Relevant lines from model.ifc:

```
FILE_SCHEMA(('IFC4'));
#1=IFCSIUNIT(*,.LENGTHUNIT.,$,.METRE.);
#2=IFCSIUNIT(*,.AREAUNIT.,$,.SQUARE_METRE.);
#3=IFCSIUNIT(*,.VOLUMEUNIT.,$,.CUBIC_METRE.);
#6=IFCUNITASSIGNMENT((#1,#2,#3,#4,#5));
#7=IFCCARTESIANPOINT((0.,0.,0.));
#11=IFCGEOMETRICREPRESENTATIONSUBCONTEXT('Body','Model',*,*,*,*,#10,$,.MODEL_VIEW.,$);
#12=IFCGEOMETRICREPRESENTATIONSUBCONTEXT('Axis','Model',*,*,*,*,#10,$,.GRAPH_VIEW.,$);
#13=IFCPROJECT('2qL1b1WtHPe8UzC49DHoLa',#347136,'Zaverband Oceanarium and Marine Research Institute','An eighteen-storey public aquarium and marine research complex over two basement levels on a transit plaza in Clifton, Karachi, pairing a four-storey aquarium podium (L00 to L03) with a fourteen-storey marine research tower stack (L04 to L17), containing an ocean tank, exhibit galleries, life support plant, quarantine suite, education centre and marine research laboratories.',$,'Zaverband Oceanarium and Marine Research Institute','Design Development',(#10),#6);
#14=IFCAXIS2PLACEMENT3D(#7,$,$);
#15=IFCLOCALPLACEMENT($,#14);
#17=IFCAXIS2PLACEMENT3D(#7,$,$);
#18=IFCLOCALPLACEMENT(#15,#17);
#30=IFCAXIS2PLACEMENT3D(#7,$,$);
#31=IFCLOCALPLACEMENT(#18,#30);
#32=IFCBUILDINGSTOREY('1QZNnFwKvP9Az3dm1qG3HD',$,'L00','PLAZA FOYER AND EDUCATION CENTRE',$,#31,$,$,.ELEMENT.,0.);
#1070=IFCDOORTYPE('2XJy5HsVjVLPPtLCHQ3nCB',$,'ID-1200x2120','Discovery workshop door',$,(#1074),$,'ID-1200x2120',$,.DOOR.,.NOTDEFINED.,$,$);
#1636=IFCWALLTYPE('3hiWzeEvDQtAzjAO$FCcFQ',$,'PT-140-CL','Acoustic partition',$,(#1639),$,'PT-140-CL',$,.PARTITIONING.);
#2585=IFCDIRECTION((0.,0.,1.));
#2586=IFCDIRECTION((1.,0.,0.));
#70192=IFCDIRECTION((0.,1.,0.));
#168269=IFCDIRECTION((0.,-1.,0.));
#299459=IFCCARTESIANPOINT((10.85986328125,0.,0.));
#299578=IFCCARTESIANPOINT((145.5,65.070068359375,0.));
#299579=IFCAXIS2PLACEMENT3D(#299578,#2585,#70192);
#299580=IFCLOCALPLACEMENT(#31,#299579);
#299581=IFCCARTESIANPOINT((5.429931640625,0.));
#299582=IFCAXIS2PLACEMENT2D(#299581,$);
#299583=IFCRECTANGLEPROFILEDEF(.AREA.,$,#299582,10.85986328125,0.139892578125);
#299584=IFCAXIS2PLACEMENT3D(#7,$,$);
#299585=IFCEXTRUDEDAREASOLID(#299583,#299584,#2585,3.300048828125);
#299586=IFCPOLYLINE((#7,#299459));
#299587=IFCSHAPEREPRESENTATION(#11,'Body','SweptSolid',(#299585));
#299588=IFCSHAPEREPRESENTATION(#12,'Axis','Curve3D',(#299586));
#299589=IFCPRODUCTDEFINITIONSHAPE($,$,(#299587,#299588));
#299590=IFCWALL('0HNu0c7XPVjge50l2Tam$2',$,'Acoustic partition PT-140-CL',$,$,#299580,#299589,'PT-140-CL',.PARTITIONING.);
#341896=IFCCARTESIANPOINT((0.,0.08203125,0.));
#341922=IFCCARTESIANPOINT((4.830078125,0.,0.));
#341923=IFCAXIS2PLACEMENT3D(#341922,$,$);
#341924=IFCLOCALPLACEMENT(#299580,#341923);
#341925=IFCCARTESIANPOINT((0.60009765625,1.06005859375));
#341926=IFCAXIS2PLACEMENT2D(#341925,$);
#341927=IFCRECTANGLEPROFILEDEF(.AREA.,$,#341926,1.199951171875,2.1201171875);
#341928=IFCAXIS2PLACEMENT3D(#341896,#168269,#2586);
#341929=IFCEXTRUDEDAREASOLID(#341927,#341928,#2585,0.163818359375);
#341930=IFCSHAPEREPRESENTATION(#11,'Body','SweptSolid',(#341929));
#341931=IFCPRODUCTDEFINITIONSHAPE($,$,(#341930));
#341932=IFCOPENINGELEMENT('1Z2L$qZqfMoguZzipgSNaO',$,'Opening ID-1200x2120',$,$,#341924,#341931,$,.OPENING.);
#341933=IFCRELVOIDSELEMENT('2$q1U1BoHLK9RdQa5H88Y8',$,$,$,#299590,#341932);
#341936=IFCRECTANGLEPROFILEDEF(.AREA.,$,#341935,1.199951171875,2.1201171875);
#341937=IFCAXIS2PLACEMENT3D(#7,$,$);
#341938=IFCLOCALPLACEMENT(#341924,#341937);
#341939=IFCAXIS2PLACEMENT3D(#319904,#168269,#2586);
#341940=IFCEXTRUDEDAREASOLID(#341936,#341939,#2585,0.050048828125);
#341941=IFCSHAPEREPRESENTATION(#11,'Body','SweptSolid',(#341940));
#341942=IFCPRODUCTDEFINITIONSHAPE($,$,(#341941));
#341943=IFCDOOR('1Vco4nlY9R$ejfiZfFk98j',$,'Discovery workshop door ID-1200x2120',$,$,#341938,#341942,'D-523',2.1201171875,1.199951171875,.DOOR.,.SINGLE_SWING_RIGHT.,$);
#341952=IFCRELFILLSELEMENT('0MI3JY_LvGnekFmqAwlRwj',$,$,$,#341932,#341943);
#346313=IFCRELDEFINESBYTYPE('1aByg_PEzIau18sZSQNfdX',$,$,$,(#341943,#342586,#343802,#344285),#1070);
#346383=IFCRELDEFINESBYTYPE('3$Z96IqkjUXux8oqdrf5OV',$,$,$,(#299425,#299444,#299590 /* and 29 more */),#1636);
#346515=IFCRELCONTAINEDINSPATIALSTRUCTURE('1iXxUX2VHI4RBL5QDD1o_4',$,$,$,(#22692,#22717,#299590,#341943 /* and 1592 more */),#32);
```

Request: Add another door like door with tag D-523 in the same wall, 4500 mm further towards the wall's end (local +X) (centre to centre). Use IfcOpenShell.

```python
import ifcopenshell
import ifcopenshell.api.feature
import ifcopenshell.api.geometry
import ifcopenshell.api.root
import ifcopenshell.geom
import ifcopenshell.util.element
import ifcopenshell.util.placement
import ifcopenshell.util.shape
import ifcopenshell.util.unit

model = ifcopenshell.open("model.ifc")
unit_scale = ifcopenshell.util.unit.calculate_unit_scale(model)
settings = ifcopenshell.geom.settings()


def volume(element):
    """Net volume in cubic metres, openings subtracted."""
    shape = ifcopenshell.geom.create_shape(settings, element)
    return ifcopenshell.util.shape.get_volume(shape.geometry)


door = model.by_guid("1Vco4nlY9R$ejfiZfFk98j")
opening = door.FillsVoids[0].RelatingOpeningElement
wall = opening.VoidsElements[0].RelatingBuildingElement
before = volume(wall)
shift = ifcopenshell.util.placement.get_local_placement(wall.ObjectPlacement)[:3, 0] * 4.5 / unit_scale

# copy_class copies the void relationship, type, container and properties, but no geometry.
new_opening = ifcopenshell.api.root.copy_class(model, product=opening)
new_opening.Representation = ifcopenshell.util.element.copy_deep(
    model, opening.Representation, exclude=["IfcGeometricRepresentationContext", "IfcRepresentationMap"]
)
new_door = ifcopenshell.api.root.copy_class(model, product=door)
new_door.Representation = ifcopenshell.util.element.copy_deep(
    model, door.Representation, exclude=["IfcGeometricRepresentationContext", "IfcRepresentationMap"]
)
new_door.Tag = None
ifcopenshell.api.feature.add_filling(model, opening=new_opening, element=new_door)

for old, new in ((opening, new_opening), (door, new_door)):
    matrix = ifcopenshell.util.placement.get_local_placement(old.ObjectPlacement)
    matrix[:3, 3] += shift
    ifcopenshell.api.geometry.edit_object_placement(model, product=new, matrix=matrix, is_si=False)

after = volume(wall)

print(f"wall volume {before:.3f} -> {after:.3f} m3")

model.write("model_updated.ifc")
```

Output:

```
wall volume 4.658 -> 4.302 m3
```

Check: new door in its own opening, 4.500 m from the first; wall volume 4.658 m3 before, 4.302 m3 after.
